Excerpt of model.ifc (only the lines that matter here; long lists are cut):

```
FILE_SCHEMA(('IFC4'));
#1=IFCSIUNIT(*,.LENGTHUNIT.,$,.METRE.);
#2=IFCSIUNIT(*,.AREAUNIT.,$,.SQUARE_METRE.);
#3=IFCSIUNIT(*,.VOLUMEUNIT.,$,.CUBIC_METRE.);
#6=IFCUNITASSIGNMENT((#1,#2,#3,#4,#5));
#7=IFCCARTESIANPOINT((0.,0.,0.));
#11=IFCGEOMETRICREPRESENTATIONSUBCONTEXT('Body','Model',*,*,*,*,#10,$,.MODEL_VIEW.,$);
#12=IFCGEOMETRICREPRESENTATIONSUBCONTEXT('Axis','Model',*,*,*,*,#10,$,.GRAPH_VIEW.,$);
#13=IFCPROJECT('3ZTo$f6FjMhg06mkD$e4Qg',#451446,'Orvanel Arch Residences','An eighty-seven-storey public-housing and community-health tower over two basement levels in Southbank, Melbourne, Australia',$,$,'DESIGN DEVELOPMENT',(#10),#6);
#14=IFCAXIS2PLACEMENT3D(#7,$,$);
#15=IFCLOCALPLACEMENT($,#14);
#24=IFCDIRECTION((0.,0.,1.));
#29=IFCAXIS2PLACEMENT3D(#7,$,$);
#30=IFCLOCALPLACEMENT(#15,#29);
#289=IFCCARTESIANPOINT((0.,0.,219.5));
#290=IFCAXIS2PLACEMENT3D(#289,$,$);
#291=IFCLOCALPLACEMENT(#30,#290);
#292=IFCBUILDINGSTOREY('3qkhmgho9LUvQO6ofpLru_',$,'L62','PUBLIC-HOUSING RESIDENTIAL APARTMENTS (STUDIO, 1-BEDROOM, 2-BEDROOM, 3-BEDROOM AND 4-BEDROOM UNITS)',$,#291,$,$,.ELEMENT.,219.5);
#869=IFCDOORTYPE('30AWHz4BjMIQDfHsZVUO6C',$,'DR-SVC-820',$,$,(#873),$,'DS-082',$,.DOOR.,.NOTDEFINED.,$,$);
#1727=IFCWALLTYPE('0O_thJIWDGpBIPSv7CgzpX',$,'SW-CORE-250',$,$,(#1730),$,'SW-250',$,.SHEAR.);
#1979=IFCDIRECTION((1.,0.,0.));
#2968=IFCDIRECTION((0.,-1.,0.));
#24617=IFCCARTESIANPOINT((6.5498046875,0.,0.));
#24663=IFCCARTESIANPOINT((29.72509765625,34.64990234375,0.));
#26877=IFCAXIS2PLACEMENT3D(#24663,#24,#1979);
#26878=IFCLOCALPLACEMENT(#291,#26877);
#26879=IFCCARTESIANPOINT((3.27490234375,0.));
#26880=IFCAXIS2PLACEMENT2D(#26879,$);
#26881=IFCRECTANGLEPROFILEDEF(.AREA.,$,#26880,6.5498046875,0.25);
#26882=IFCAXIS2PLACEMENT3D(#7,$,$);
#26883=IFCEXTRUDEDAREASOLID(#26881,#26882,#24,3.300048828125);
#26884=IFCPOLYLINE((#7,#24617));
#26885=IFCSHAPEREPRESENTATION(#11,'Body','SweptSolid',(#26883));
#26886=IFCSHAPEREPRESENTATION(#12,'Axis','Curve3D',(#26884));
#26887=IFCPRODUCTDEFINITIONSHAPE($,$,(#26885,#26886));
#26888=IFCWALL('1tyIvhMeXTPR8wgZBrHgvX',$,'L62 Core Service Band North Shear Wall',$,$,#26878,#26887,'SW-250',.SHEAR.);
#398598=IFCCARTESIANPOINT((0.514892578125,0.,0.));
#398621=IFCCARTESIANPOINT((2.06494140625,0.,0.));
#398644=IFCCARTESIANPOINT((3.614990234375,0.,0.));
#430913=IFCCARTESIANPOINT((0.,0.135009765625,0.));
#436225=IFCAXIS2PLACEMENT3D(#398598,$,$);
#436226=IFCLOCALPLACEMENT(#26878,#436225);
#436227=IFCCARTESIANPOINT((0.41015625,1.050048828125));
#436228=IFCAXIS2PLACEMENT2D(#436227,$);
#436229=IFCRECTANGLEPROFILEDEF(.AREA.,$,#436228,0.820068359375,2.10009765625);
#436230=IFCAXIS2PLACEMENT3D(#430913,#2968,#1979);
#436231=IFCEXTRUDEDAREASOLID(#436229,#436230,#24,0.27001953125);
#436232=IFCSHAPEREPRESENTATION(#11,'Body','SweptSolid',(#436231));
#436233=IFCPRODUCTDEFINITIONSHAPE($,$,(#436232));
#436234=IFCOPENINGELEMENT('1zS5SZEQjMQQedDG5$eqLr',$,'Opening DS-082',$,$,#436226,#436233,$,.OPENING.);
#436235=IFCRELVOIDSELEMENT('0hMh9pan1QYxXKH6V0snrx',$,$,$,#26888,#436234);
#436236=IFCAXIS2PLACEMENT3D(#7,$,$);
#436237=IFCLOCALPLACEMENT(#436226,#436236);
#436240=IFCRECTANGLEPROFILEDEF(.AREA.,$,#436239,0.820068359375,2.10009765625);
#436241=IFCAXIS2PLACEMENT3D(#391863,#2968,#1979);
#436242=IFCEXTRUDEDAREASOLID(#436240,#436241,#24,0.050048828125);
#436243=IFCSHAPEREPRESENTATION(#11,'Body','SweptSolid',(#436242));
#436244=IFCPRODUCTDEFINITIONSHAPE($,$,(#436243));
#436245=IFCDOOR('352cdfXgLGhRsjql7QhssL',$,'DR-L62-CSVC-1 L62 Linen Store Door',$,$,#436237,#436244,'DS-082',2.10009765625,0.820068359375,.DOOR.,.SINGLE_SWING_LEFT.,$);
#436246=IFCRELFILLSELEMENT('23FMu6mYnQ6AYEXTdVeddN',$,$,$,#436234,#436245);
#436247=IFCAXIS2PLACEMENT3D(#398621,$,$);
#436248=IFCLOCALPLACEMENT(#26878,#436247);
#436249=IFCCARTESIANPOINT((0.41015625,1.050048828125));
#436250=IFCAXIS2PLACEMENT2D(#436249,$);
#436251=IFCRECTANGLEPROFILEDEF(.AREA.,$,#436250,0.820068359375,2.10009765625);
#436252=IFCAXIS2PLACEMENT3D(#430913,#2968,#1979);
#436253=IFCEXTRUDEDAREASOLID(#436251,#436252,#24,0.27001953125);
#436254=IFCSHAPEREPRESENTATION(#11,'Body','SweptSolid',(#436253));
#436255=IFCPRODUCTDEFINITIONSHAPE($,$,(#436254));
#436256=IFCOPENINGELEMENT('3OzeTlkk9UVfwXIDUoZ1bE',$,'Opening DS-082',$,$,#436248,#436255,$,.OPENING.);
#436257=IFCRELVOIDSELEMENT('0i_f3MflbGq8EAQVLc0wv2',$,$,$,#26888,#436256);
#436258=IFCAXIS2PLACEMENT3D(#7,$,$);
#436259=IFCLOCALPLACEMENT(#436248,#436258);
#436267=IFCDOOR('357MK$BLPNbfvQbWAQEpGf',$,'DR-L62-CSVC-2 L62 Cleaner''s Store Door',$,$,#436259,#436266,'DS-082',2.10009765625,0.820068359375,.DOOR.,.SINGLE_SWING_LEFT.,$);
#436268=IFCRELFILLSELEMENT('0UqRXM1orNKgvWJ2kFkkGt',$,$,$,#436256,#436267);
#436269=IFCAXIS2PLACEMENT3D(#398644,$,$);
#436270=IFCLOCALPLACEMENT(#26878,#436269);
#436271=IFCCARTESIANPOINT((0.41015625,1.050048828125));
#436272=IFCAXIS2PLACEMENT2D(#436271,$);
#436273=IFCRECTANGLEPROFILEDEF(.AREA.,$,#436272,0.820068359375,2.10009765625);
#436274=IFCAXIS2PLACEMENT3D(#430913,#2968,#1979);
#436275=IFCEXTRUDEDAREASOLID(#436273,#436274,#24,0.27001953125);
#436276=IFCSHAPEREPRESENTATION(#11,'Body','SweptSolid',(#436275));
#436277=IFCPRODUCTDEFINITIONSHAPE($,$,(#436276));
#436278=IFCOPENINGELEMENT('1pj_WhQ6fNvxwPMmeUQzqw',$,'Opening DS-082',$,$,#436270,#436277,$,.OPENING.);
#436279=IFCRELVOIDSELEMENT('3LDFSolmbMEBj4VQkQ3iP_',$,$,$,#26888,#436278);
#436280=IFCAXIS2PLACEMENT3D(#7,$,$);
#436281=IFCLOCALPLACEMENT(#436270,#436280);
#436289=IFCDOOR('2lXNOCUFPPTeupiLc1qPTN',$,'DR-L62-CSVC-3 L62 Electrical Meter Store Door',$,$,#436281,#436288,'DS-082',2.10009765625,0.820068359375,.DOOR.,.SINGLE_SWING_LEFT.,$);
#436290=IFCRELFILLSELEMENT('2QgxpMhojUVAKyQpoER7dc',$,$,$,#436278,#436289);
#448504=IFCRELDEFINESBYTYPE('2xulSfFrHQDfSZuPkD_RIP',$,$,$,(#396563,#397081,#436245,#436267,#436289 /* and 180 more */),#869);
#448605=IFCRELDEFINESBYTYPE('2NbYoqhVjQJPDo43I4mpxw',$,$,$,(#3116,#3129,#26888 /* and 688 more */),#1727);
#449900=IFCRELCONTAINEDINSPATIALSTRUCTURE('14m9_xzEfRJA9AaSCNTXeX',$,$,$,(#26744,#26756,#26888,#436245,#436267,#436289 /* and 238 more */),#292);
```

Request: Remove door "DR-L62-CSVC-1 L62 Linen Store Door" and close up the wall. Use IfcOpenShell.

```python
import ifcopenshell
import ifcopenshell.api.feature
import ifcopenshell.api.root
import ifcopenshell.geom
import ifcopenshell.util.shape

model = ifcopenshell.open("model.ifc")
settings = ifcopenshell.geom.settings()


def volume(element):
    """Net volume in cubic metres, openings subtracted."""
    shape = ifcopenshell.geom.create_shape(settings, element)
    return ifcopenshell.util.shape.get_volume(shape.geometry)


door = model.by_guid("352cdfXgLGhRsjql7QhssL")
opening = door.FillsVoids[0].RelatingOpeningElement
wall = opening.VoidsElements[0].RelatingBuildingElement
before = volume(wall)

ifcopenshell.api.root.remove_product(model, product=door)
ifcopenshell.api.feature.remove_feature(model, feature=opening)

after = volume(wall)

print(f"wall volume {before:.3f} -> {after:.3f} m3")

model.write("model-out.ifc")
```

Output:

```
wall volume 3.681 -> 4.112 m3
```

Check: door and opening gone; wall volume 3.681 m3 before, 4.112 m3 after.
